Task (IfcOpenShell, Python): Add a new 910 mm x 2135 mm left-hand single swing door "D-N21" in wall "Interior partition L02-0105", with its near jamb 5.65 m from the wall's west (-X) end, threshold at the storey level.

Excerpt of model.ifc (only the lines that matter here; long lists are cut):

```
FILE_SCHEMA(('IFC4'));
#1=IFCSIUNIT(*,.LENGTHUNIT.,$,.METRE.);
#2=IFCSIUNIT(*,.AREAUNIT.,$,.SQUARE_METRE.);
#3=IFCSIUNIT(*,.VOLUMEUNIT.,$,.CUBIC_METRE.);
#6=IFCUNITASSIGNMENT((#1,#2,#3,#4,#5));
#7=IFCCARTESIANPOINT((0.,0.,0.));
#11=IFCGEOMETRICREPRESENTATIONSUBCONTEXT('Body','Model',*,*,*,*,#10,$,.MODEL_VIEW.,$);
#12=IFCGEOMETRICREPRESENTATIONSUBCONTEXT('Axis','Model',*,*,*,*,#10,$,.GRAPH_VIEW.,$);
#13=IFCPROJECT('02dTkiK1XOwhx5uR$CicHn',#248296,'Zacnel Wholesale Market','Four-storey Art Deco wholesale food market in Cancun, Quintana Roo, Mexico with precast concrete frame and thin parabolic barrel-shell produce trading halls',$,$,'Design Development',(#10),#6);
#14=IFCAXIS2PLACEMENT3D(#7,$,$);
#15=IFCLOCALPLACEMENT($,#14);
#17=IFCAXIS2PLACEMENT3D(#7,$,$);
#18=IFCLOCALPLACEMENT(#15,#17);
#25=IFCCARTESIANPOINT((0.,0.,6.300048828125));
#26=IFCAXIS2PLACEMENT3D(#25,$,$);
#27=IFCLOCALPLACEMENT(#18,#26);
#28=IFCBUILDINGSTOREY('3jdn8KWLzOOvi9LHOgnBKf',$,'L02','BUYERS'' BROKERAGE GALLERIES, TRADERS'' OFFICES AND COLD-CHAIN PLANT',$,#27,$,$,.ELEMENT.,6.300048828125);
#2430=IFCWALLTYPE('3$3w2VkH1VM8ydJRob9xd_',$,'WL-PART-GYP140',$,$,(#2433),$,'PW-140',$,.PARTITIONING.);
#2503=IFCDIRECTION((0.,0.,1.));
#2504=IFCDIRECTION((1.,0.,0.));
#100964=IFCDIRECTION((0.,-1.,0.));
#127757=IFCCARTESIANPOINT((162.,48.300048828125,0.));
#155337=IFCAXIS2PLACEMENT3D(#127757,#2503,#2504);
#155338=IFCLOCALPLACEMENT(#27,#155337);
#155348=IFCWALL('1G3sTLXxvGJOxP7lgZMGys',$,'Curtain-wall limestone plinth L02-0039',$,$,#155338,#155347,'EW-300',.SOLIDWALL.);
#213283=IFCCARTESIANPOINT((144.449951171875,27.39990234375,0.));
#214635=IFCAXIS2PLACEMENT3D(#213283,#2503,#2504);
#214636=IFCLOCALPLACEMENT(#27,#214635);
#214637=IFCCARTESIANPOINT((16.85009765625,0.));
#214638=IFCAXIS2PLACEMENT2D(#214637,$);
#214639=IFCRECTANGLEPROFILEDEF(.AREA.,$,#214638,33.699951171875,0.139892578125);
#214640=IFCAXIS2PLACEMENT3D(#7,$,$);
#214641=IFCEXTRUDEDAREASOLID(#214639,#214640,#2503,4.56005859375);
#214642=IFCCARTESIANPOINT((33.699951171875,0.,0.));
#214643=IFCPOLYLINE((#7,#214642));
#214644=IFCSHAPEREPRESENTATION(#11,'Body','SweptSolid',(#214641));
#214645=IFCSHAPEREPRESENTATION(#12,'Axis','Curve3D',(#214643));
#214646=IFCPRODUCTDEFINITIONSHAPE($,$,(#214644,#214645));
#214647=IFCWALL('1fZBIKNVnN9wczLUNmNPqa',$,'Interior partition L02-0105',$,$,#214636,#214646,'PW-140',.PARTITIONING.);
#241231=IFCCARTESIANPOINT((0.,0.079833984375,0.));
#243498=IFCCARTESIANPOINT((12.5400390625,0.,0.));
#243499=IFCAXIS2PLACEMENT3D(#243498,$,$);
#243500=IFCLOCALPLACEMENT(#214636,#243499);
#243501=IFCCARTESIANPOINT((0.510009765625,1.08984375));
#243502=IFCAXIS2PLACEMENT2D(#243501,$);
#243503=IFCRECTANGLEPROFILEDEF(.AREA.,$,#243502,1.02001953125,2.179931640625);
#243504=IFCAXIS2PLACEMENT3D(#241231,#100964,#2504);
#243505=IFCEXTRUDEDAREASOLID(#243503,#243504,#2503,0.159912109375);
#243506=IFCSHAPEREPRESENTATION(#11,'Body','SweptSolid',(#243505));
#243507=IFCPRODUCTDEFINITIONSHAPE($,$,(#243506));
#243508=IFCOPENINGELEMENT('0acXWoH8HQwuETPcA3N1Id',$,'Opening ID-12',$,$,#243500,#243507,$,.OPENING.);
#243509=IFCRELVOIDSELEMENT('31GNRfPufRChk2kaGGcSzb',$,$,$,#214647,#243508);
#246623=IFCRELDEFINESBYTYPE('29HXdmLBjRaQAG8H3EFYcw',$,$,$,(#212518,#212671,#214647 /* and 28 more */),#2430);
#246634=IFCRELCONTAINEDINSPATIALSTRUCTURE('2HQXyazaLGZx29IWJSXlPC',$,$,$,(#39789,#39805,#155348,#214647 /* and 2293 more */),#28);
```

```python
import numpy as np
import ifcopenshell
import ifcopenshell.api.feature
import ifcopenshell.api.geometry
import ifcopenshell.api.root
import ifcopenshell.api.spatial
import ifcopenshell.geom
import ifcopenshell.util.element
import ifcopenshell.util.placement
import ifcopenshell.util.representation
import ifcopenshell.util.shape
import ifcopenshell.util.unit

model = ifcopenshell.open("model.ifc")
unit_scale = ifcopenshell.util.unit.calculate_unit_scale(model)
settings = ifcopenshell.geom.settings()


def volume(element):
    """Net volume in cubic metres, openings subtracted."""
    shape = ifcopenshell.geom.create_shape(settings, element)
    return ifcopenshell.util.shape.get_volume(shape.geometry)


wall = model.by_guid("1fZBIKNVnN9wczLUNmNPqa")
storey = ifcopenshell.util.element.get_container(wall, ifc_class="IfcBuildingStorey")
context = ifcopenshell.util.representation.get_context(model, "Model", "Body", "MODEL_VIEW")
before = volume(wall)

width, height, from_end, sill = 0.91, 2.135, 5.65, 0.0  # metres

# The wall runs along its own X axis, and the end named is its -X end.
wall_shape = ifcopenshell.geom.create_shape(settings, wall)
x, y, z = ifcopenshell.util.shape.get_vertices(wall_shape.geometry).T
start = x.min() + from_end
face, thickness = float(y.min()), float(y.max() - y.min())
wall_matrix = ifcopenshell.util.placement.get_local_placement(wall.ObjectPlacement)
level = ifcopenshell.util.placement.get_local_placement(storey.ObjectPlacement)[2, 3]


def in_wall(x, y):
    """Placement at x, y metres in the wall's axes, at sill height."""
    matrix = wall_matrix.copy()
    matrix[:, 3] = wall_matrix @ np.array([x / unit_scale, y / unit_scale, 0.0, 1.0])
    matrix[2, 3] = level + sill / unit_scale
    return matrix


# Opening: a box that overshoots both wall faces by 50 mm.
opening = ifcopenshell.api.root.create_entity(model, ifc_class="IfcOpeningElement", predefined_type="OPENING")
box = ifcopenshell.api.geometry.add_wall_representation(
    model, context=context, length=width, height=height, thickness=thickness + 0.1
)
ifcopenshell.api.geometry.assign_representation(model, product=opening, representation=box)
ifcopenshell.api.geometry.edit_object_placement(model, product=opening, matrix=in_wall(start, face - 0.05), is_si=False)
ifcopenshell.api.feature.add_feature(model, feature=opening, element=wall)

door = ifcopenshell.api.root.create_entity(model, ifc_class="IfcDoor", name="D-N21", predefined_type="DOOR")
door.OverallWidth, door.OverallHeight = width / unit_scale, height / unit_scale
door.OperationType = "SINGLE_SWING_LEFT"
body = ifcopenshell.api.geometry.add_door_representation(
    model,
    context=context,
    overall_width=door.OverallWidth,
    overall_height=door.OverallHeight,
    operation_type="SINGLE_SWING_LEFT",
    lining_properties={"LiningDepth": thickness / unit_scale, "ThresholdDepth": thickness / unit_scale},
)
ifcopenshell.api.geometry.assign_representation(model, product=door, representation=body)
ifcopenshell.api.spatial.assign_container(model, products=[door], relating_structure=storey)
ifcopenshell.api.feature.add_filling(model, opening=opening, element=door)

# The lining spans the wall, so the door starts at the wall face.
ifcopenshell.api.geometry.edit_object_placement(model, product=door, matrix=in_wall(start, face), is_si=False)

after = volume(wall)

print(f"wall volume {before:.3f} -> {after:.3f} m3")

model.write("model-out.ifc")
```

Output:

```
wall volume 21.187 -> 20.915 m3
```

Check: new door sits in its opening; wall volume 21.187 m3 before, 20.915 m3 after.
